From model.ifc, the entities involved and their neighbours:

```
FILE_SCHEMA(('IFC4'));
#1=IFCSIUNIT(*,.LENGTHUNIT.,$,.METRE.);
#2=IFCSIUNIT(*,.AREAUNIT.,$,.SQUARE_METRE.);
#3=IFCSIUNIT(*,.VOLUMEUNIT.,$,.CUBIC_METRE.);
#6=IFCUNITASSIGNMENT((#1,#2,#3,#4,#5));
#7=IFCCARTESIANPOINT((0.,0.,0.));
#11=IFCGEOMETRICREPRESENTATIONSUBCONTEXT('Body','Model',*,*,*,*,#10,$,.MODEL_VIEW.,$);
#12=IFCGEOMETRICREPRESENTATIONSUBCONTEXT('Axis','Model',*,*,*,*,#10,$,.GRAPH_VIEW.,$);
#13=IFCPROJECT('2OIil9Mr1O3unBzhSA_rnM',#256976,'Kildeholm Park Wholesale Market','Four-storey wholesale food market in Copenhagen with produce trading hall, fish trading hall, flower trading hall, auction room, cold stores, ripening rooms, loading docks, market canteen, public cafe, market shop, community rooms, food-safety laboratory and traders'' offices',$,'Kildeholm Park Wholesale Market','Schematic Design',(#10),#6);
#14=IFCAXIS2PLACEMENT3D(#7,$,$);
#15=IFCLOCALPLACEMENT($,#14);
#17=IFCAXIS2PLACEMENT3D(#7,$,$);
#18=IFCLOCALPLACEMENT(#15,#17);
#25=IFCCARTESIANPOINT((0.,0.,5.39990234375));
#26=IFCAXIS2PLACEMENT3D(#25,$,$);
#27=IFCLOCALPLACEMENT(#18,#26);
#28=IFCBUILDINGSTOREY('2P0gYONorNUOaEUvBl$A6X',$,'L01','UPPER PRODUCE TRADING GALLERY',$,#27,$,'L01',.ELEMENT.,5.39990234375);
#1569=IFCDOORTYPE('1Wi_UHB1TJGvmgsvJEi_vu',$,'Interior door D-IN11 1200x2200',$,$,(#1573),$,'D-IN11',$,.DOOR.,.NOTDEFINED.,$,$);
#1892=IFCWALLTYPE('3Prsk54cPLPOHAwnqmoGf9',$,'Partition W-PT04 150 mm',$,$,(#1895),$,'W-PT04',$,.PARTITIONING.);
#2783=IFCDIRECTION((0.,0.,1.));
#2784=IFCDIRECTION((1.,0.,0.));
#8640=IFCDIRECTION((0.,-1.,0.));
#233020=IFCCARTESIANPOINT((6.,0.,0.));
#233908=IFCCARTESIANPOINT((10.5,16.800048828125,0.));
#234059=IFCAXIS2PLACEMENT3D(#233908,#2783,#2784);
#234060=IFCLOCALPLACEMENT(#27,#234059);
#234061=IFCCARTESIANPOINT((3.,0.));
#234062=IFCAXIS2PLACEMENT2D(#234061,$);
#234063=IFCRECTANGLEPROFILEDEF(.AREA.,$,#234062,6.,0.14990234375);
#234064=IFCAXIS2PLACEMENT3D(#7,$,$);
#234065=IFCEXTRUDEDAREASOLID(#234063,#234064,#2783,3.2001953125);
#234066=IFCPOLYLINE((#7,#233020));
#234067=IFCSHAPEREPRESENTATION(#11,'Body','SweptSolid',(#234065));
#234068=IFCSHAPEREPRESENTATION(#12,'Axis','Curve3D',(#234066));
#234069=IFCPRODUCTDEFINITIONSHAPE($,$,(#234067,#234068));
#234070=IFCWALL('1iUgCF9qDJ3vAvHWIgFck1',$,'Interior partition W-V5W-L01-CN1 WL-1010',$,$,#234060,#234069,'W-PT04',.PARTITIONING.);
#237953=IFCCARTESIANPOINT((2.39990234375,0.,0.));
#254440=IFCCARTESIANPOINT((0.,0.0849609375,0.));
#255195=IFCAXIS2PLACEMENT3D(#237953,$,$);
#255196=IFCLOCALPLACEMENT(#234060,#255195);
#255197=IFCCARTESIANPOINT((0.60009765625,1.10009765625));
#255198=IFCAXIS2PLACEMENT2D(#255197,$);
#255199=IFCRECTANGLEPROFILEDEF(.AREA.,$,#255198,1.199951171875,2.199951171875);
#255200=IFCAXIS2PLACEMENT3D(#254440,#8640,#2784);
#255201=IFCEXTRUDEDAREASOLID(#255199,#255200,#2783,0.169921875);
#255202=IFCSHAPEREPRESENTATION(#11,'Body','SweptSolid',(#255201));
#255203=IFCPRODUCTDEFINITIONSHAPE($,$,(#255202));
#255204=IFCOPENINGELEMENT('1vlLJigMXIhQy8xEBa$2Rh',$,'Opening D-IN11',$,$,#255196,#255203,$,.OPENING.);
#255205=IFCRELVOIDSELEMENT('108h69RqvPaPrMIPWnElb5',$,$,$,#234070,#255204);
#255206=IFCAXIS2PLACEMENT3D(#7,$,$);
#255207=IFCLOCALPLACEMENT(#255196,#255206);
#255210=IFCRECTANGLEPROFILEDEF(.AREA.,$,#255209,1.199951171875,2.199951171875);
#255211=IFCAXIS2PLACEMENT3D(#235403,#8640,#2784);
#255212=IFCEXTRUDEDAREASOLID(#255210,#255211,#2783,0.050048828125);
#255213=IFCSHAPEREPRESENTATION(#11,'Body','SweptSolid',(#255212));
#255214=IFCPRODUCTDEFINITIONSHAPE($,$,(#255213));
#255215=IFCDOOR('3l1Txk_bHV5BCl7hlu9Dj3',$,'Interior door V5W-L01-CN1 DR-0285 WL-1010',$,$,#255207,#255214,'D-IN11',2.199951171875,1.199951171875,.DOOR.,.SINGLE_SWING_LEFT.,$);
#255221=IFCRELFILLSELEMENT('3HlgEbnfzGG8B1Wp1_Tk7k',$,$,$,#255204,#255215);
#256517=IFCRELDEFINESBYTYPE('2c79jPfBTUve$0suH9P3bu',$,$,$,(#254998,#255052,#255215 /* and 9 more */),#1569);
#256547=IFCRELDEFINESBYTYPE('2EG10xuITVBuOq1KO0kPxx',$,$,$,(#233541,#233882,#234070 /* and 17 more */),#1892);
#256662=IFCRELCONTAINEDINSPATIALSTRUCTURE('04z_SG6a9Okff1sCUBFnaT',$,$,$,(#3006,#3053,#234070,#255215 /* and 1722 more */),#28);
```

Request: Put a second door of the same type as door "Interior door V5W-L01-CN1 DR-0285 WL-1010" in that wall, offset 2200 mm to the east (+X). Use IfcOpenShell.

```python
import ifcopenshell
import ifcopenshell.api.feature
import ifcopenshell.api.geometry
import ifcopenshell.api.root
import ifcopenshell.geom
import ifcopenshell.util.element
import ifcopenshell.util.placement
import ifcopenshell.util.shape

model = ifcopenshell.open("model.ifc")
settings = ifcopenshell.geom.settings()


def volume(element):
    """Net volume in cubic metres, openings subtracted."""
    shape = ifcopenshell.geom.create_shape(settings, element)
    return ifcopenshell.util.shape.get_volume(shape.geometry)


door = model.by_guid("3l1Txk_bHV5BCl7hlu9Dj3")
opening = door.FillsVoids[0].RelatingOpeningElement
wall = opening.VoidsElements[0].RelatingBuildingElement
before = volume(wall)
shift = ifcopenshell.util.placement.get_local_placement(wall.ObjectPlacement)[:3, 0] * 2.2

# copy_class copies the void relationship, type, container and properties, but no geometry.
new_opening = ifcopenshell.api.root.copy_class(model, product=opening)
new_opening.Representation = ifcopenshell.util.element.copy_deep(
    model, opening.Representation, exclude=["IfcGeometricRepresentationContext", "IfcRepresentationMap"]
)
new_door = ifcopenshell.api.root.copy_class(model, product=door)
new_door.Representation = ifcopenshell.util.element.copy_deep(
    model, door.Representation, exclude=["IfcGeometricRepresentationContext", "IfcRepresentationMap"]
)
new_door.Tag = None
ifcopenshell.api.feature.add_filling(model, opening=new_opening, element=new_door)

for old, new in ((opening, new_opening), (door, new_door)):
    matrix = ifcopenshell.util.placement.get_local_placement(old.ObjectPlacement)
    matrix[:3, 3] += shift
    ifcopenshell.api.geometry.edit_object_placement(model, product=new, matrix=matrix, is_si=False)

after = volume(wall)

print(f"wall volume {before:.3f} -> {after:.3f} m3")

model.write("model_v2.ifc")
```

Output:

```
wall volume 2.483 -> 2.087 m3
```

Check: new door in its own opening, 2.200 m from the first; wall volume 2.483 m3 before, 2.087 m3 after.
